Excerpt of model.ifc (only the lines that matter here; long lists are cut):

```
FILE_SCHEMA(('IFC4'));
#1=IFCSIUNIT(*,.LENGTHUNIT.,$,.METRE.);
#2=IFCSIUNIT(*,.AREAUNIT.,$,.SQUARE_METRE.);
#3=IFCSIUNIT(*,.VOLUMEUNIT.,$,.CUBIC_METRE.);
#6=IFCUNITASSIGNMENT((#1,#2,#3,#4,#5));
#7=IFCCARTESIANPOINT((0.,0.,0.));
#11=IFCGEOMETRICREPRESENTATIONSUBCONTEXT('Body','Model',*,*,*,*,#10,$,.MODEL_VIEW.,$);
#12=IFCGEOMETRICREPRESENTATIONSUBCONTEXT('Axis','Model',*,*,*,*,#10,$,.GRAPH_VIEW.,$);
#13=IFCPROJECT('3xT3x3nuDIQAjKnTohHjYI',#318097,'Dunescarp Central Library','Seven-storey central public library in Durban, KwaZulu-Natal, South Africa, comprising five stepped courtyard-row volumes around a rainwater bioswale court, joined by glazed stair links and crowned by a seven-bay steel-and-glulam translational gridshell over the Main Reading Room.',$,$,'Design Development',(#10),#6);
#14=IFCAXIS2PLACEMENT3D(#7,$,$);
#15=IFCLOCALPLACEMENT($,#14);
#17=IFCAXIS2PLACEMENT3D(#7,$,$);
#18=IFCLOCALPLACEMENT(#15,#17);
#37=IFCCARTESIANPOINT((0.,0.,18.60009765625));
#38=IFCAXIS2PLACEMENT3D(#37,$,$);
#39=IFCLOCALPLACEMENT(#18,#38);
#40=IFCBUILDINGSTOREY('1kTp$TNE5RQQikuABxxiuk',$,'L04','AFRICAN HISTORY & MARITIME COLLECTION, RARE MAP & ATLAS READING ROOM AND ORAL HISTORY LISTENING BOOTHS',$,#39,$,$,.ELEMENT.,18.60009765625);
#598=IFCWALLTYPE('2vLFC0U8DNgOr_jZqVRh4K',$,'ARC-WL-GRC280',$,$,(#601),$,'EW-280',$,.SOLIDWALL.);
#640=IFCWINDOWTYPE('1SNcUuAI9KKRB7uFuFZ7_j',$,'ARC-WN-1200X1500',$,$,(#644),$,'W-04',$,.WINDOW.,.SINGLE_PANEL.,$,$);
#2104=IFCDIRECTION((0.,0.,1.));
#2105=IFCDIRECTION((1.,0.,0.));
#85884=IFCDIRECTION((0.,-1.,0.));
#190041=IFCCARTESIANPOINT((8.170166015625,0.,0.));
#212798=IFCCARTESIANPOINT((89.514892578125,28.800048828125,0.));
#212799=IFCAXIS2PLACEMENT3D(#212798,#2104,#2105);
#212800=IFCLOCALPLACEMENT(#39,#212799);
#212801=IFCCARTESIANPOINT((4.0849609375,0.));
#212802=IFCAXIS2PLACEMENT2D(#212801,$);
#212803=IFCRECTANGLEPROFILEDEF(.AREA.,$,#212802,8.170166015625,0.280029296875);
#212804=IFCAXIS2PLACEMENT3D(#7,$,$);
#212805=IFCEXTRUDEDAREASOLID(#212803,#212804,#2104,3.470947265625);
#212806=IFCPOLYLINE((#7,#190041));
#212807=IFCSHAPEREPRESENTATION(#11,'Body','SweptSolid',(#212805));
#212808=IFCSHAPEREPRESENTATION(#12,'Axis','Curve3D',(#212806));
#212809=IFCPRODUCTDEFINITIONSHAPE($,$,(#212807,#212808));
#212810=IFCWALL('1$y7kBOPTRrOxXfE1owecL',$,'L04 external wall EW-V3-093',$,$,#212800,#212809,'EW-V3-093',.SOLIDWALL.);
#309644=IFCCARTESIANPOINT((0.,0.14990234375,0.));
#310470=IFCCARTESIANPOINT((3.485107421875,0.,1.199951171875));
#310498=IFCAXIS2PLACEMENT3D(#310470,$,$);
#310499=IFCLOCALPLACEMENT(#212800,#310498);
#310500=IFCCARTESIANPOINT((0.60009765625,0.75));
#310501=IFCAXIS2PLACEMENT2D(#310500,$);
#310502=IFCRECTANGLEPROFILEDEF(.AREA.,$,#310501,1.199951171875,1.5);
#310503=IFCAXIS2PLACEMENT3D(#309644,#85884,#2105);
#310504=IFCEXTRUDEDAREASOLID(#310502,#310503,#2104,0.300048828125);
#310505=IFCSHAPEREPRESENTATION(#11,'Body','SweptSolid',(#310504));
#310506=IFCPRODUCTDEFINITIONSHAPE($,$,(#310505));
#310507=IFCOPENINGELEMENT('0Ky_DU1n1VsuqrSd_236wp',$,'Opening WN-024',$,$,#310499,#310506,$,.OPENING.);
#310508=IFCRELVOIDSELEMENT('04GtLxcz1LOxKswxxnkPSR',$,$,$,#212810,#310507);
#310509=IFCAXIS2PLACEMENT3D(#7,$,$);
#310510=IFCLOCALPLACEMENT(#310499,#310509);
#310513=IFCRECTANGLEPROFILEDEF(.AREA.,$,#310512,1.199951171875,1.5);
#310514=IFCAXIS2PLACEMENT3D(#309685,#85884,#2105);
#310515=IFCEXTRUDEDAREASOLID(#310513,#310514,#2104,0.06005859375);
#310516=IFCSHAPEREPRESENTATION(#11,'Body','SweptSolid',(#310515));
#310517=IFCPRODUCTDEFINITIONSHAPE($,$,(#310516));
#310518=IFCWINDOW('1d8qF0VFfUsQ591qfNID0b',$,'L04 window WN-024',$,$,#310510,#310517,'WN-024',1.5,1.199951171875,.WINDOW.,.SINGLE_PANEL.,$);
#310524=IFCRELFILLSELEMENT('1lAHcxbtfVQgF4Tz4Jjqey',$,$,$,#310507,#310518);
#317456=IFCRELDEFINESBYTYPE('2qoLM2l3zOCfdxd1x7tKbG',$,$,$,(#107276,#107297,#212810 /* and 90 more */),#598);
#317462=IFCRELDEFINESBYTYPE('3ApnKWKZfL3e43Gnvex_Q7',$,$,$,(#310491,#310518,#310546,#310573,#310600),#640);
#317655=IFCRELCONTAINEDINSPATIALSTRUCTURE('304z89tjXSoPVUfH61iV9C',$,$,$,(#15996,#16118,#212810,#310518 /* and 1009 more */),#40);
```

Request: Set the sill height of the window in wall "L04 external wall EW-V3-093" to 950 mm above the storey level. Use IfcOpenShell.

```python
import numpy as np
import ifcopenshell
import ifcopenshell.api.geometry
import ifcopenshell.geom
import ifcopenshell.util.element
import ifcopenshell.util.placement
import ifcopenshell.util.shape
import ifcopenshell.util.unit

model = ifcopenshell.open("model.ifc")
unit_scale = ifcopenshell.util.unit.calculate_unit_scale(model)

window = model.by_id(310518)
opening = window.FillsVoids[0].RelatingOpeningElement
storey = ifcopenshell.util.element.get_container(window, ifc_class="IfcBuildingStorey")
level = ifcopenshell.util.placement.get_local_placement(storey.ObjectPlacement)[2, 3]

# The opening's origin need not be at the sill, so measure its lowest point.
shape = ifcopenshell.geom.create_shape(ifcopenshell.geom.settings(), opening)
bottom = ifcopenshell.util.shape.get_shape_bottom_elevation(shape, shape.geometry) / unit_scale
dz = level + 0.95 / unit_scale - bottom

shift = np.array([0.0, 0.0, dz])
# The window is placed relative to its opening, so it follows when the opening moves.
matrix = ifcopenshell.util.placement.get_local_placement(opening.ObjectPlacement)
matrix[:3, 3] += shift
ifcopenshell.api.geometry.edit_object_placement(
    model, product=opening, matrix=matrix, is_si=False, should_transform_children=True
)

print(f"moved by {dz * unit_scale:+.3f} m")

model.write("model_edited.ifc")
```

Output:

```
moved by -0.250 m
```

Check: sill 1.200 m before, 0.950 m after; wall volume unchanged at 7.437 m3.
